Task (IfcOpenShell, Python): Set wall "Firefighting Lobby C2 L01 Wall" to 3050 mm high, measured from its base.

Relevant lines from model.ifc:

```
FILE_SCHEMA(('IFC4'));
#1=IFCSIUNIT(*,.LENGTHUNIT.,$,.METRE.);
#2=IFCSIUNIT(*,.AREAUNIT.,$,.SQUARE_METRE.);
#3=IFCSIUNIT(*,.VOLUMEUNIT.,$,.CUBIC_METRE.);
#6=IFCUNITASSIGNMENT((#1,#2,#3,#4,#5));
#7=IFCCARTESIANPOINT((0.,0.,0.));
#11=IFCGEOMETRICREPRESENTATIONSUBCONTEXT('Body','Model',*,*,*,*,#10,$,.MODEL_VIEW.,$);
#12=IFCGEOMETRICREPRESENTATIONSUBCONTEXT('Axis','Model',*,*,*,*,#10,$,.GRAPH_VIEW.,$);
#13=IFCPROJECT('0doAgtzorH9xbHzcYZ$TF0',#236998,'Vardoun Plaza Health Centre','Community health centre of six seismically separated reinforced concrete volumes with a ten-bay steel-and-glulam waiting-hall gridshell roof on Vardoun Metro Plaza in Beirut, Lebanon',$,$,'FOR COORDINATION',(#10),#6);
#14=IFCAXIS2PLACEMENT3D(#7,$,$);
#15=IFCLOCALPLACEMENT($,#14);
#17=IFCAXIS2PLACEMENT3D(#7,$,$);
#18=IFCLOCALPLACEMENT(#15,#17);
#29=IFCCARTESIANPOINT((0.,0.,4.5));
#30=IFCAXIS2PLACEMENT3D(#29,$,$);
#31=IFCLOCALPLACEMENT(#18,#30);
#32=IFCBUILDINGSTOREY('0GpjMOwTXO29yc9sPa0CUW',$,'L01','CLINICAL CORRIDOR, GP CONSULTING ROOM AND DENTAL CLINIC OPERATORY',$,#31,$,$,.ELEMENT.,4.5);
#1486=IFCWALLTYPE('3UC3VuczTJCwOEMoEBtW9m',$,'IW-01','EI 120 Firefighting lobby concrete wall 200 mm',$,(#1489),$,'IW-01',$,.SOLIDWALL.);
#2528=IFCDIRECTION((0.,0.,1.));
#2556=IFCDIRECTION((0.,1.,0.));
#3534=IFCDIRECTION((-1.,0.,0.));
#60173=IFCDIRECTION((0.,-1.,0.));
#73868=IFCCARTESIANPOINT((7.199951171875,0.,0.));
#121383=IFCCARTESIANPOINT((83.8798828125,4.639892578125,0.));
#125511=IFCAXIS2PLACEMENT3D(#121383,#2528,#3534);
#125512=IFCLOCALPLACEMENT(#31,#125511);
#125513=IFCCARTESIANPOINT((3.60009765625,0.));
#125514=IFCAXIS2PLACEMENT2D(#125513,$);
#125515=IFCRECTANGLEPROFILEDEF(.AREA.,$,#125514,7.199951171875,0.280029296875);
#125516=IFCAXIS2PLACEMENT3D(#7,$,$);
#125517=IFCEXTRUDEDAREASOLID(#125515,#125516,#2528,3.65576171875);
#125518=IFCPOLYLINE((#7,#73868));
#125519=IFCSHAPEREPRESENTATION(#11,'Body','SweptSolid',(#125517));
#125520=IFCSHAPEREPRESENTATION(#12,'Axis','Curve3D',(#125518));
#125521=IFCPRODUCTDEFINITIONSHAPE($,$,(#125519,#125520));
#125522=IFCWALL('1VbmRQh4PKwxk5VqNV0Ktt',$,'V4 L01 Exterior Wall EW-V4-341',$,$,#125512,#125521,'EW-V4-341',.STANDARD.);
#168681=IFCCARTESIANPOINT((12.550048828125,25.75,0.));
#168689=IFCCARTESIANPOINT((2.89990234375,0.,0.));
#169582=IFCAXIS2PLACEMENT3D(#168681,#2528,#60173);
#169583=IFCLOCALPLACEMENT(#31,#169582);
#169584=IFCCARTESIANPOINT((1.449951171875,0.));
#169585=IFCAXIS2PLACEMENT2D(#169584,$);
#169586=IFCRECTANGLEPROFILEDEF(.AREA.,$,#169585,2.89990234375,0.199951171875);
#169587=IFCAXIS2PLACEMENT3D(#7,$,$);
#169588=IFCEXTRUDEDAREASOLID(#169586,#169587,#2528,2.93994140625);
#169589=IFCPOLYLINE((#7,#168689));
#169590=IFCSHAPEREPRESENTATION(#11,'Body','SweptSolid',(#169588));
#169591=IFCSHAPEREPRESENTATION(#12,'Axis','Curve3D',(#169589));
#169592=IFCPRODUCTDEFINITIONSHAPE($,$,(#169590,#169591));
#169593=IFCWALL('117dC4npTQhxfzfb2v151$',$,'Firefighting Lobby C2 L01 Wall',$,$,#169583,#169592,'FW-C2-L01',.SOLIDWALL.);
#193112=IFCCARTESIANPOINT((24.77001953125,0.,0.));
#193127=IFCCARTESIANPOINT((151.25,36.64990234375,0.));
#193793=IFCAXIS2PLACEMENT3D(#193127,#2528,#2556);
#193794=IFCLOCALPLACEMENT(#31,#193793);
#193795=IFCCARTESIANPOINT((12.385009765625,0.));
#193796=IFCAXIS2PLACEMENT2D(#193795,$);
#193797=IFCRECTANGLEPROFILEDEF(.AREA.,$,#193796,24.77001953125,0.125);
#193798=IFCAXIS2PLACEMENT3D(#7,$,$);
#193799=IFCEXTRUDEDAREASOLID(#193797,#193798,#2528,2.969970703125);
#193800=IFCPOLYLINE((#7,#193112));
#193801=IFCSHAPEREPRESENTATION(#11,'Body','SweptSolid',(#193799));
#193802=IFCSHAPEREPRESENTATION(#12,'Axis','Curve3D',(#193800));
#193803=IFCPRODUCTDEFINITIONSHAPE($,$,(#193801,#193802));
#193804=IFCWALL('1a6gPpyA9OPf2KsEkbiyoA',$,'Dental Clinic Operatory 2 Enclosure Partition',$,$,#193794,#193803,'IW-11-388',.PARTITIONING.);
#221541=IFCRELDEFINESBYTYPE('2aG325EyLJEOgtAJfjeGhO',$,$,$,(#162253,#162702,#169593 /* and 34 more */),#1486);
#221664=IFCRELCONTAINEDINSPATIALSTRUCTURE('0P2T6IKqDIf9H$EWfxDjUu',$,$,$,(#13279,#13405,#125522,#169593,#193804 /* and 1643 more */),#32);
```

```python
import ifcopenshell
import ifcopenshell.geom
import ifcopenshell.util.representation
import ifcopenshell.util.shape
import ifcopenshell.util.unit

model = ifcopenshell.open("model.ifc")
unit_scale = ifcopenshell.util.unit.calculate_unit_scale(model)
settings = ifcopenshell.geom.settings()


def volume(element):
    """Net volume in cubic metres, openings subtracted."""
    shape = ifcopenshell.geom.create_shape(settings, element)
    return ifcopenshell.util.shape.get_volume(shape.geometry)


wall = model.by_guid("117dC4npTQhxfzfb2v151$")
before = volume(wall)

body = ifcopenshell.util.representation.get_representation(wall, "Model", "Body")
solid = body.Items[0]
old_height = solid.Depth
solid.Depth = 3.05 / unit_scale
after = volume(wall)

print(f"height {old_height:g} -> {solid.Depth:g}, volume {before:.3f} -> {after:.3f} m3")

model.write("model-out.ifc")
```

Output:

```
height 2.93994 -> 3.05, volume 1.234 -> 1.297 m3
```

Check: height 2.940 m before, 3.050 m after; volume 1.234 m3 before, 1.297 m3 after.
